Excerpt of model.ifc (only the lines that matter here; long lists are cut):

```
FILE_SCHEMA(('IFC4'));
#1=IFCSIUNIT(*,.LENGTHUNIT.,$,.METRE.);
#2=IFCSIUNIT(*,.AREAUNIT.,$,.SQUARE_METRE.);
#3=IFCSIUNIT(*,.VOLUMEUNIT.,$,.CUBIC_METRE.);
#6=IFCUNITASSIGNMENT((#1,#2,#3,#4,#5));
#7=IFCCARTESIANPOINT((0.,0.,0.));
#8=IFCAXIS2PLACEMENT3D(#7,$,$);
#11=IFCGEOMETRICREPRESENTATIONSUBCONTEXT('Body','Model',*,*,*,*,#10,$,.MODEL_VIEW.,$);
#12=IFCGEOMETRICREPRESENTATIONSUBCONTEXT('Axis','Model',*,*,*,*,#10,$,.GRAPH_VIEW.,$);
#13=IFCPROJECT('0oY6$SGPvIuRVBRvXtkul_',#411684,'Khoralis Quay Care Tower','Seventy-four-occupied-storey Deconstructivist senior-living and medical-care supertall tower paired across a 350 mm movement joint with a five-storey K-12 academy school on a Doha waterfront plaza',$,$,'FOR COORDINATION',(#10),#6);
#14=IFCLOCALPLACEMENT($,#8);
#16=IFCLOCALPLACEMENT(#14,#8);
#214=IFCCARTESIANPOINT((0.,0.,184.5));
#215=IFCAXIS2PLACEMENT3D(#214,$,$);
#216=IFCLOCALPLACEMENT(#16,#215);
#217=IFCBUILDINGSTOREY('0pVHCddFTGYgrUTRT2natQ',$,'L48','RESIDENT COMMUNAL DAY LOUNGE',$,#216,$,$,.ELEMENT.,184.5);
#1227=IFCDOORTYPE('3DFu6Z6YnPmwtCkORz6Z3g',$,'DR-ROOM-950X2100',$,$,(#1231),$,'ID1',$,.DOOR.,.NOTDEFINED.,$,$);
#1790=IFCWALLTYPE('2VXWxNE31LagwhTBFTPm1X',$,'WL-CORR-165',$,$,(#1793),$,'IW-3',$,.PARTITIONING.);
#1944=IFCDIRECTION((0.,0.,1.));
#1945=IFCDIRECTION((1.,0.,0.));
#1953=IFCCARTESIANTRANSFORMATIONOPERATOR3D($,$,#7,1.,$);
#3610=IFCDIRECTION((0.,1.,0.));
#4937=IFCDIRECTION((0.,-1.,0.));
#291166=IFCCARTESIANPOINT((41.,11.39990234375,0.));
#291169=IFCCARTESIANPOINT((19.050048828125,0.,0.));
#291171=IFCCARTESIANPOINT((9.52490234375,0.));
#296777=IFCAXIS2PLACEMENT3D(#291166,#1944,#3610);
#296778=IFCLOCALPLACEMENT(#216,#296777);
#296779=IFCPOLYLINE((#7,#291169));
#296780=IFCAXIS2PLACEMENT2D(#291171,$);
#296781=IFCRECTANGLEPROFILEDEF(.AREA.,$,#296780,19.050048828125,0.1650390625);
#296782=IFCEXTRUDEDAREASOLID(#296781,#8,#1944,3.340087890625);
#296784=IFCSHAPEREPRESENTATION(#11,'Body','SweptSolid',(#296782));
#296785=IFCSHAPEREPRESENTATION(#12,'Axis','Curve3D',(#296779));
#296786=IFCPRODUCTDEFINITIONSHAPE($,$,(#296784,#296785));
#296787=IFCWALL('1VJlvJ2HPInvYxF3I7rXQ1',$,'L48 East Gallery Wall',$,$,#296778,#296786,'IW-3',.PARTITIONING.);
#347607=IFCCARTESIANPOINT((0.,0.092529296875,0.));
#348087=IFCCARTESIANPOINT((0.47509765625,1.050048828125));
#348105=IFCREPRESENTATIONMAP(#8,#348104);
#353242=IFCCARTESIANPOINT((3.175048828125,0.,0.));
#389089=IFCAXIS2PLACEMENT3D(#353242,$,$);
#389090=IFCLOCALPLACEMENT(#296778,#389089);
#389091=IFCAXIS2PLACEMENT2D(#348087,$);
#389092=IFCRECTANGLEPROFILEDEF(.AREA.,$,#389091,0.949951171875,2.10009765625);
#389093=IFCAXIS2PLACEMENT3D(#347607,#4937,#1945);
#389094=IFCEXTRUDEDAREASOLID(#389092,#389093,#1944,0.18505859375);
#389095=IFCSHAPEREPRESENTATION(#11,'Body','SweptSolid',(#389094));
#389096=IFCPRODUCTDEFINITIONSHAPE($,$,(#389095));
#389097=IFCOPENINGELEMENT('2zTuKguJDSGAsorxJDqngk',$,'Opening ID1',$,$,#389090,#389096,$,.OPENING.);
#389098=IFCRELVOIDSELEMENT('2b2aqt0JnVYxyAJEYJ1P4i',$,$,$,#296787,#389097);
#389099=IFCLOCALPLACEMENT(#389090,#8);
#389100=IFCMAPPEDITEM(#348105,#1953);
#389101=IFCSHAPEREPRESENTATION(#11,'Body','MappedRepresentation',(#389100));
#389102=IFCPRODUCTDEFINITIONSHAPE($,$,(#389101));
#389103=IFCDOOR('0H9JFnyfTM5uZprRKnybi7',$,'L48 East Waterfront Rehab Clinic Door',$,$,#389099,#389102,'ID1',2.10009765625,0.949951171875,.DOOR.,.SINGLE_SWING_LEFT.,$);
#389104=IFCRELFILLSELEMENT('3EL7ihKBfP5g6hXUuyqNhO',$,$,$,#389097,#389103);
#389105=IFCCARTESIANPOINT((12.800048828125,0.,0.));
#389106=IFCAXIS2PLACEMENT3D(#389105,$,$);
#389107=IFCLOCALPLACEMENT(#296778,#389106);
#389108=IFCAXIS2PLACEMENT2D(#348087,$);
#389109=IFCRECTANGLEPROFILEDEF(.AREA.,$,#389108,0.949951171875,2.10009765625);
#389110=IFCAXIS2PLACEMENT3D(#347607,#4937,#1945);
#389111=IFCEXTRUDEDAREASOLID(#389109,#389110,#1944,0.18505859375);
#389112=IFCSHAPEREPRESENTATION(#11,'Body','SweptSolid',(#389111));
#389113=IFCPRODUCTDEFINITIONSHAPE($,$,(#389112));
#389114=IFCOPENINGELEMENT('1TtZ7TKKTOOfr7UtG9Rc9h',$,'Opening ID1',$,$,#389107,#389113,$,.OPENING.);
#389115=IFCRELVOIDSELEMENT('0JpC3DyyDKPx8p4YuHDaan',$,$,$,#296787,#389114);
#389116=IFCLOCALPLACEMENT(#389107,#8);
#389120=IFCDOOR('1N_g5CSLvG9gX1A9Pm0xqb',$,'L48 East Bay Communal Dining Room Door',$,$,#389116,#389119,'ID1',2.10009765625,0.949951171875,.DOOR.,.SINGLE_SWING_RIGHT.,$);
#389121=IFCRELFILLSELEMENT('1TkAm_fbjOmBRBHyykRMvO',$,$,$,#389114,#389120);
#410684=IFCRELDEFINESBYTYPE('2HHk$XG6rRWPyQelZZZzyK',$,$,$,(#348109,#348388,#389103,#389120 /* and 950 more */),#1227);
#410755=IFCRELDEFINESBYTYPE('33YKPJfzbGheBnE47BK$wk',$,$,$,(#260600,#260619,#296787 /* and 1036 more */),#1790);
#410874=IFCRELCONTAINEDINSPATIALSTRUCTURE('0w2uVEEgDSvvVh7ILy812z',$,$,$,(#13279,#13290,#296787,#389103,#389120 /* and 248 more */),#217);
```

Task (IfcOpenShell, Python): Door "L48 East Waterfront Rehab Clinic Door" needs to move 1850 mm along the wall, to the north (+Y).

```python
import ifcopenshell
import ifcopenshell.api.geometry
import ifcopenshell.util.placement
import ifcopenshell.util.unit

model = ifcopenshell.open("model.ifc")
unit_scale = ifcopenshell.util.unit.calculate_unit_scale(model)

door = model.by_guid("0H9JFnyfTM5uZprRKnybi7")
opening = door.FillsVoids[0].RelatingOpeningElement
wall = opening.VoidsElements[0].RelatingBuildingElement

wall_matrix = ifcopenshell.util.placement.get_local_placement(wall.ObjectPlacement)
shift = wall_matrix[:3, 0] * 1.85 / unit_scale
before = ifcopenshell.util.placement.get_local_placement(door.ObjectPlacement)[:3, 3].copy()

# The door is placed relative to its opening, so it follows when the opening moves.
matrix = ifcopenshell.util.placement.get_local_placement(opening.ObjectPlacement)
matrix[:3, 3] += shift
ifcopenshell.api.geometry.edit_object_placement(
    model, product=opening, matrix=matrix, is_si=False, should_transform_children=True
)

after = ifcopenshell.util.placement.get_local_placement(door.ObjectPlacement)[:3, 3]
print("door moved by", (after - before).round(3) + 0.0)

model.write("model_v2.ifc")
```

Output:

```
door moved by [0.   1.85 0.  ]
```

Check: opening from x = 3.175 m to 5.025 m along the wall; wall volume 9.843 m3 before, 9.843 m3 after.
